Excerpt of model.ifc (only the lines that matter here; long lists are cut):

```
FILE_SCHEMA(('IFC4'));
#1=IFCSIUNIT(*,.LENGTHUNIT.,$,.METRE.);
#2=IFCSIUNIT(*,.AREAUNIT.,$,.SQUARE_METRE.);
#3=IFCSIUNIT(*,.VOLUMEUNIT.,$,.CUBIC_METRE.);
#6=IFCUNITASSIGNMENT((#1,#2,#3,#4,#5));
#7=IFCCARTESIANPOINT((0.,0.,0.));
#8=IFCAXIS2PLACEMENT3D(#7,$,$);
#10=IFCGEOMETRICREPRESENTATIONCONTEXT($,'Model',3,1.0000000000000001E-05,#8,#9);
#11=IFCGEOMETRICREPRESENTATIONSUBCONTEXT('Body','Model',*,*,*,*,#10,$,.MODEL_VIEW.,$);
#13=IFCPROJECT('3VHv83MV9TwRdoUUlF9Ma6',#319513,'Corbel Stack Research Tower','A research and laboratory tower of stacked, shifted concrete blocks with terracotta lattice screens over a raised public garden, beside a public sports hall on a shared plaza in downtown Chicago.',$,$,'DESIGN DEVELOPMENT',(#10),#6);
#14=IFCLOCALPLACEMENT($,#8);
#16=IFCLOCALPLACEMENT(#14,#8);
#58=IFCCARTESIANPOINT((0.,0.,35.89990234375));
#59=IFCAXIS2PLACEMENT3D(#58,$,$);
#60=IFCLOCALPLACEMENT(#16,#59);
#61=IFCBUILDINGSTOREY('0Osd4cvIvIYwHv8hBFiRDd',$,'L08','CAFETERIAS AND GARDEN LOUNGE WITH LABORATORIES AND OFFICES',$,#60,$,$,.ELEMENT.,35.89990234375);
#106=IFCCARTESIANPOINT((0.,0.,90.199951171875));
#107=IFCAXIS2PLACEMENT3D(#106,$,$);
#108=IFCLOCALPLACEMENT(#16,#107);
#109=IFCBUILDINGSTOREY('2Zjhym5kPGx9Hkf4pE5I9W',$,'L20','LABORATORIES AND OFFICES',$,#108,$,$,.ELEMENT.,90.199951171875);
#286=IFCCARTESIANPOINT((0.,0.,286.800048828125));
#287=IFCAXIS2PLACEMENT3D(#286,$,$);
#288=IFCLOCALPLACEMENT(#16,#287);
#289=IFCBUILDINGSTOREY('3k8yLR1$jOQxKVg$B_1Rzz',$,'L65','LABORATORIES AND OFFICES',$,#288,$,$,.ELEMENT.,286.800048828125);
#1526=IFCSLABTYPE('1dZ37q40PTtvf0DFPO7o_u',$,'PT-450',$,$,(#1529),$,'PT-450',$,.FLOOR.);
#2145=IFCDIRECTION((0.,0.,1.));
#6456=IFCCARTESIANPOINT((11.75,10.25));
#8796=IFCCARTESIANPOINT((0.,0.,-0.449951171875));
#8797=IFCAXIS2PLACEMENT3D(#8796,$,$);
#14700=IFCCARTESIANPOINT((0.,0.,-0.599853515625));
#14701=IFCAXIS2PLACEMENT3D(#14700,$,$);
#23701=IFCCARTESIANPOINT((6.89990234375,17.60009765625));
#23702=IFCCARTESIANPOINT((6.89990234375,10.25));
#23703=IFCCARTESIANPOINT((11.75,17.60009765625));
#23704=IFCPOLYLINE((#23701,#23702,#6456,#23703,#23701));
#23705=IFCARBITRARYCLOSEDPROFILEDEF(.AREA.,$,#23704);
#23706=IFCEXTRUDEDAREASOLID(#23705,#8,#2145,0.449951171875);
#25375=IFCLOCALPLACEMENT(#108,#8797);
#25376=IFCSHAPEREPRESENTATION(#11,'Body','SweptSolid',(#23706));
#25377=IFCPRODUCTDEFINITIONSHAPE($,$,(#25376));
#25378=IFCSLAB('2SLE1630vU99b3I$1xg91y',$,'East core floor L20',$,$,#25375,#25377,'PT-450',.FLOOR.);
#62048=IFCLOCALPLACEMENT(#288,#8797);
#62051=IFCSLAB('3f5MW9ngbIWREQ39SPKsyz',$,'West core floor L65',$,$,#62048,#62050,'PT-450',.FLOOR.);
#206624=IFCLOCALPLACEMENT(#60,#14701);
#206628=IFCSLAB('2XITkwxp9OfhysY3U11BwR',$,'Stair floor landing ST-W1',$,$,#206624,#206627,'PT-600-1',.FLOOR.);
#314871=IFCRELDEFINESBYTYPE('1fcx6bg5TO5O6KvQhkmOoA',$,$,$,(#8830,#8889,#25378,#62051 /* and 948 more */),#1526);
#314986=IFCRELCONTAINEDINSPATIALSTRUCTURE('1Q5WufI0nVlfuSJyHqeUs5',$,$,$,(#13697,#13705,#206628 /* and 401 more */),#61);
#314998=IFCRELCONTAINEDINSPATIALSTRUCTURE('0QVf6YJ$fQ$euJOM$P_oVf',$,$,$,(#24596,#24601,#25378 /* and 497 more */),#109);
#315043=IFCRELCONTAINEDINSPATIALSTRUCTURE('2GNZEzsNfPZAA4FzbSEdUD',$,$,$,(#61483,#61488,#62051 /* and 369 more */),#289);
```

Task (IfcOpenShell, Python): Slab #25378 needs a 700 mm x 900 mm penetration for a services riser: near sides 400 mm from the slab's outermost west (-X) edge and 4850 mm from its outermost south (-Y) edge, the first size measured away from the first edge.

```python
import numpy as np
import ifcopenshell
import ifcopenshell.api.feature
import ifcopenshell.api.geometry
import ifcopenshell.api.root
import ifcopenshell.geom
import ifcopenshell.util.placement
import ifcopenshell.util.representation
import ifcopenshell.util.shape
import ifcopenshell.util.unit

model = ifcopenshell.open("model.ifc")
unit_scale = ifcopenshell.util.unit.calculate_unit_scale(model)
settings = ifcopenshell.geom.settings()


def volume(element):
    """Net volume in cubic metres, openings subtracted."""
    shape = ifcopenshell.geom.create_shape(settings, element)
    return ifcopenshell.util.shape.get_volume(shape.geometry)


slab = model.by_guid("2SLE1630vU99b3I$1xg91y")
before = volume(slab)

# Extent in the slab's own axes, in metres. The edges named are its -X and -Y sides.
slab_shape = ifcopenshell.geom.create_shape(settings, slab)
vertices = ifcopenshell.util.shape.get_vertices(slab_shape.geometry)
x_min, y_min, bottom = vertices.min(axis=0)
top = vertices[:, 2].max()

opening = ifcopenshell.api.root.create_entity(model, ifc_class="IfcOpeningElement", name="Services riser opening", predefined_type="OPENING")
context = ifcopenshell.util.representation.get_context(model, "Model", "Body", "MODEL_VIEW")
width, depth = 0.7, 0.9
outline = [(0.0, 0.0), (width, 0.0), (width, depth), (0.0, depth), (0.0, 0.0)]
# Overshoot both faces by 50 mm so the cut is clean.
shape = ifcopenshell.api.geometry.add_slab_representation(
    model, context=context, depth=top - bottom + 0.1, polyline=outline
)
ifcopenshell.api.geometry.assign_representation(model, product=opening, representation=shape)

matrix = ifcopenshell.util.placement.get_local_placement(slab.ObjectPlacement)
matrix[:, 3] = matrix @ np.append(np.array([x_min + 0.4, y_min + 4.85, bottom - 0.05]) / unit_scale, 1.0)
ifcopenshell.api.geometry.edit_object_placement(model, product=opening, matrix=matrix, is_si=False)
ifcopenshell.api.feature.add_feature(model, feature=opening, element=slab)

after = volume(slab)

print(f"slab volume {before:.3f} -> {after:.3f} m3")

model.write("model_updated.ifc")
```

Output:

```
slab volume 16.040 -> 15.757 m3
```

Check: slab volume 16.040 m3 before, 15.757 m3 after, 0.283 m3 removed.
